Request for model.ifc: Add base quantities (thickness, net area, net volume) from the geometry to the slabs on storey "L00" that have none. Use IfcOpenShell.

First a look at what the model holds.

```python
import ifcopenshell
import ifcopenshell.util.element
import ifcopenshell.util.unit

model = ifcopenshell.open("model.ifc")
print(model.schema)
for unit_type in ("LENGTHUNIT", "AREAUNIT", "VOLUMEUNIT"):
    print(unit_type, ifcopenshell.util.unit.calculate_unit_scale(model, unit_type))
storey = next(s for s in model.by_type("IfcBuildingStorey") if s.Name == "L00")
slabs = [e for e in ifcopenshell.util.element.get_decomposition(storey) if e.is_a("IfcSlab")]
for e in sorted(slabs, key=lambda e: e.id()):
    print(e.id(), e.is_a(), e.Name, list(ifcopenshell.util.element.get_psets(e, qtos_only=True)), sep=" | ")
```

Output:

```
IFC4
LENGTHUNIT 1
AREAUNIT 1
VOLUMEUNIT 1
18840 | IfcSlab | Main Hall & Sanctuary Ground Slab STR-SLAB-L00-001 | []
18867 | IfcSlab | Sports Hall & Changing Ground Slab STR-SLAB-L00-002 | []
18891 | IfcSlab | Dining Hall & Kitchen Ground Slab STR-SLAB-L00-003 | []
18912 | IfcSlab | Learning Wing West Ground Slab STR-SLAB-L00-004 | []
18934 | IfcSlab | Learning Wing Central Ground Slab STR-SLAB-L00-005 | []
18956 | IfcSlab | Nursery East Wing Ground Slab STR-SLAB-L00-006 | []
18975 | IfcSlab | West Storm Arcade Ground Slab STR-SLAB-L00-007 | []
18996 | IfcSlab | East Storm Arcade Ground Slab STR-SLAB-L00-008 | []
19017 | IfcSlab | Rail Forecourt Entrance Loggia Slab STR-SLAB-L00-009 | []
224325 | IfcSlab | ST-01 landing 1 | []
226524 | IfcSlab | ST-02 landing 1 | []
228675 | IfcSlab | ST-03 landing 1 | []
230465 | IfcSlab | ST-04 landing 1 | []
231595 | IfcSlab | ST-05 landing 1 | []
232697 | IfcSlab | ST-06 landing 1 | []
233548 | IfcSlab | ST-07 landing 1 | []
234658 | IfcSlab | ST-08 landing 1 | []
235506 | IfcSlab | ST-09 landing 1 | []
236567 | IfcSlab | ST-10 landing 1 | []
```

```python
import ifcopenshell
import ifcopenshell.api.pset
import ifcopenshell.geom
import ifcopenshell.util.element
import ifcopenshell.util.shape
import ifcopenshell.util.unit

model = ifcopenshell.open("model.ifc")
unit_scale = ifcopenshell.util.unit.calculate_unit_scale(model)
area_scale = ifcopenshell.util.unit.calculate_unit_scale(model, "AREAUNIT")
volume_scale = ifcopenshell.util.unit.calculate_unit_scale(model, "VOLUMEUNIT")
settings = ifcopenshell.geom.settings()

storey = next(s for s in model.by_type("IfcBuildingStorey") if s.Name == "L00")
slabs = [e for e in ifcopenshell.util.element.get_decomposition(storey) if e.is_a("IfcSlab")]

for e in sorted(slabs, key=lambda e: e.id()):
    if ifcopenshell.util.element.get_psets(e, qtos_only=True, should_inherit=False):
        continue
    # Geometry comes back in metres, in the element's own axes.
    shape = ifcopenshell.geom.create_shape(settings, e)
    values = {
        "Width": ifcopenshell.util.shape.get_z(shape.geometry) / unit_scale,
        "NetArea": ifcopenshell.util.shape.get_footprint_area(shape.geometry) / area_scale,
        "NetVolume": ifcopenshell.util.shape.get_volume(shape.geometry) / volume_scale,
    }
    qto = ifcopenshell.api.pset.add_qto(model, product=e, name="Qto_SlabBaseQuantities")
    ifcopenshell.api.pset.edit_qto(model, qto=qto, properties=values)
    print(e.id(), {k: round(v, 3) for k, v in values.items()})

model.write("model_rev.ifc")
```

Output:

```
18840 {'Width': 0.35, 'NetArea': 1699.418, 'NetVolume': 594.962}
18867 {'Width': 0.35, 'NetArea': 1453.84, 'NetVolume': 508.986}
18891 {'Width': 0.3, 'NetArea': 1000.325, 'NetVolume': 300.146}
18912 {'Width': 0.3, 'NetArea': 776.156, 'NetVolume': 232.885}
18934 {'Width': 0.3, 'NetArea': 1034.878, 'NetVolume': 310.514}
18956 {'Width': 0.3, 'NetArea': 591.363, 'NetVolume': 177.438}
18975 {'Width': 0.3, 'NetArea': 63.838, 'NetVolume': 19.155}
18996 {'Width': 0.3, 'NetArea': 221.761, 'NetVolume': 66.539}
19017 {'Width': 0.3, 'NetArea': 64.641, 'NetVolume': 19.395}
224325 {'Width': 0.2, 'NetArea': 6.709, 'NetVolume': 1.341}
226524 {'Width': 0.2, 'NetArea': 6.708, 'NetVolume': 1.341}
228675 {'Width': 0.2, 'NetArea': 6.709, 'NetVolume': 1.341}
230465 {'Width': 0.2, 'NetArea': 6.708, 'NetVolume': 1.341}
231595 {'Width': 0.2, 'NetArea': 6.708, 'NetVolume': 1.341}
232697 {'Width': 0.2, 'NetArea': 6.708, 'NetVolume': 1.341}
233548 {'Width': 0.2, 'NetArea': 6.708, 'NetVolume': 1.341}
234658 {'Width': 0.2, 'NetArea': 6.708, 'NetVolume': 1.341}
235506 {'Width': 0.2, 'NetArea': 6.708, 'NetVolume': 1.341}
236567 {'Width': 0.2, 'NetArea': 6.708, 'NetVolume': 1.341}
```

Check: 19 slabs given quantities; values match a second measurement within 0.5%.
